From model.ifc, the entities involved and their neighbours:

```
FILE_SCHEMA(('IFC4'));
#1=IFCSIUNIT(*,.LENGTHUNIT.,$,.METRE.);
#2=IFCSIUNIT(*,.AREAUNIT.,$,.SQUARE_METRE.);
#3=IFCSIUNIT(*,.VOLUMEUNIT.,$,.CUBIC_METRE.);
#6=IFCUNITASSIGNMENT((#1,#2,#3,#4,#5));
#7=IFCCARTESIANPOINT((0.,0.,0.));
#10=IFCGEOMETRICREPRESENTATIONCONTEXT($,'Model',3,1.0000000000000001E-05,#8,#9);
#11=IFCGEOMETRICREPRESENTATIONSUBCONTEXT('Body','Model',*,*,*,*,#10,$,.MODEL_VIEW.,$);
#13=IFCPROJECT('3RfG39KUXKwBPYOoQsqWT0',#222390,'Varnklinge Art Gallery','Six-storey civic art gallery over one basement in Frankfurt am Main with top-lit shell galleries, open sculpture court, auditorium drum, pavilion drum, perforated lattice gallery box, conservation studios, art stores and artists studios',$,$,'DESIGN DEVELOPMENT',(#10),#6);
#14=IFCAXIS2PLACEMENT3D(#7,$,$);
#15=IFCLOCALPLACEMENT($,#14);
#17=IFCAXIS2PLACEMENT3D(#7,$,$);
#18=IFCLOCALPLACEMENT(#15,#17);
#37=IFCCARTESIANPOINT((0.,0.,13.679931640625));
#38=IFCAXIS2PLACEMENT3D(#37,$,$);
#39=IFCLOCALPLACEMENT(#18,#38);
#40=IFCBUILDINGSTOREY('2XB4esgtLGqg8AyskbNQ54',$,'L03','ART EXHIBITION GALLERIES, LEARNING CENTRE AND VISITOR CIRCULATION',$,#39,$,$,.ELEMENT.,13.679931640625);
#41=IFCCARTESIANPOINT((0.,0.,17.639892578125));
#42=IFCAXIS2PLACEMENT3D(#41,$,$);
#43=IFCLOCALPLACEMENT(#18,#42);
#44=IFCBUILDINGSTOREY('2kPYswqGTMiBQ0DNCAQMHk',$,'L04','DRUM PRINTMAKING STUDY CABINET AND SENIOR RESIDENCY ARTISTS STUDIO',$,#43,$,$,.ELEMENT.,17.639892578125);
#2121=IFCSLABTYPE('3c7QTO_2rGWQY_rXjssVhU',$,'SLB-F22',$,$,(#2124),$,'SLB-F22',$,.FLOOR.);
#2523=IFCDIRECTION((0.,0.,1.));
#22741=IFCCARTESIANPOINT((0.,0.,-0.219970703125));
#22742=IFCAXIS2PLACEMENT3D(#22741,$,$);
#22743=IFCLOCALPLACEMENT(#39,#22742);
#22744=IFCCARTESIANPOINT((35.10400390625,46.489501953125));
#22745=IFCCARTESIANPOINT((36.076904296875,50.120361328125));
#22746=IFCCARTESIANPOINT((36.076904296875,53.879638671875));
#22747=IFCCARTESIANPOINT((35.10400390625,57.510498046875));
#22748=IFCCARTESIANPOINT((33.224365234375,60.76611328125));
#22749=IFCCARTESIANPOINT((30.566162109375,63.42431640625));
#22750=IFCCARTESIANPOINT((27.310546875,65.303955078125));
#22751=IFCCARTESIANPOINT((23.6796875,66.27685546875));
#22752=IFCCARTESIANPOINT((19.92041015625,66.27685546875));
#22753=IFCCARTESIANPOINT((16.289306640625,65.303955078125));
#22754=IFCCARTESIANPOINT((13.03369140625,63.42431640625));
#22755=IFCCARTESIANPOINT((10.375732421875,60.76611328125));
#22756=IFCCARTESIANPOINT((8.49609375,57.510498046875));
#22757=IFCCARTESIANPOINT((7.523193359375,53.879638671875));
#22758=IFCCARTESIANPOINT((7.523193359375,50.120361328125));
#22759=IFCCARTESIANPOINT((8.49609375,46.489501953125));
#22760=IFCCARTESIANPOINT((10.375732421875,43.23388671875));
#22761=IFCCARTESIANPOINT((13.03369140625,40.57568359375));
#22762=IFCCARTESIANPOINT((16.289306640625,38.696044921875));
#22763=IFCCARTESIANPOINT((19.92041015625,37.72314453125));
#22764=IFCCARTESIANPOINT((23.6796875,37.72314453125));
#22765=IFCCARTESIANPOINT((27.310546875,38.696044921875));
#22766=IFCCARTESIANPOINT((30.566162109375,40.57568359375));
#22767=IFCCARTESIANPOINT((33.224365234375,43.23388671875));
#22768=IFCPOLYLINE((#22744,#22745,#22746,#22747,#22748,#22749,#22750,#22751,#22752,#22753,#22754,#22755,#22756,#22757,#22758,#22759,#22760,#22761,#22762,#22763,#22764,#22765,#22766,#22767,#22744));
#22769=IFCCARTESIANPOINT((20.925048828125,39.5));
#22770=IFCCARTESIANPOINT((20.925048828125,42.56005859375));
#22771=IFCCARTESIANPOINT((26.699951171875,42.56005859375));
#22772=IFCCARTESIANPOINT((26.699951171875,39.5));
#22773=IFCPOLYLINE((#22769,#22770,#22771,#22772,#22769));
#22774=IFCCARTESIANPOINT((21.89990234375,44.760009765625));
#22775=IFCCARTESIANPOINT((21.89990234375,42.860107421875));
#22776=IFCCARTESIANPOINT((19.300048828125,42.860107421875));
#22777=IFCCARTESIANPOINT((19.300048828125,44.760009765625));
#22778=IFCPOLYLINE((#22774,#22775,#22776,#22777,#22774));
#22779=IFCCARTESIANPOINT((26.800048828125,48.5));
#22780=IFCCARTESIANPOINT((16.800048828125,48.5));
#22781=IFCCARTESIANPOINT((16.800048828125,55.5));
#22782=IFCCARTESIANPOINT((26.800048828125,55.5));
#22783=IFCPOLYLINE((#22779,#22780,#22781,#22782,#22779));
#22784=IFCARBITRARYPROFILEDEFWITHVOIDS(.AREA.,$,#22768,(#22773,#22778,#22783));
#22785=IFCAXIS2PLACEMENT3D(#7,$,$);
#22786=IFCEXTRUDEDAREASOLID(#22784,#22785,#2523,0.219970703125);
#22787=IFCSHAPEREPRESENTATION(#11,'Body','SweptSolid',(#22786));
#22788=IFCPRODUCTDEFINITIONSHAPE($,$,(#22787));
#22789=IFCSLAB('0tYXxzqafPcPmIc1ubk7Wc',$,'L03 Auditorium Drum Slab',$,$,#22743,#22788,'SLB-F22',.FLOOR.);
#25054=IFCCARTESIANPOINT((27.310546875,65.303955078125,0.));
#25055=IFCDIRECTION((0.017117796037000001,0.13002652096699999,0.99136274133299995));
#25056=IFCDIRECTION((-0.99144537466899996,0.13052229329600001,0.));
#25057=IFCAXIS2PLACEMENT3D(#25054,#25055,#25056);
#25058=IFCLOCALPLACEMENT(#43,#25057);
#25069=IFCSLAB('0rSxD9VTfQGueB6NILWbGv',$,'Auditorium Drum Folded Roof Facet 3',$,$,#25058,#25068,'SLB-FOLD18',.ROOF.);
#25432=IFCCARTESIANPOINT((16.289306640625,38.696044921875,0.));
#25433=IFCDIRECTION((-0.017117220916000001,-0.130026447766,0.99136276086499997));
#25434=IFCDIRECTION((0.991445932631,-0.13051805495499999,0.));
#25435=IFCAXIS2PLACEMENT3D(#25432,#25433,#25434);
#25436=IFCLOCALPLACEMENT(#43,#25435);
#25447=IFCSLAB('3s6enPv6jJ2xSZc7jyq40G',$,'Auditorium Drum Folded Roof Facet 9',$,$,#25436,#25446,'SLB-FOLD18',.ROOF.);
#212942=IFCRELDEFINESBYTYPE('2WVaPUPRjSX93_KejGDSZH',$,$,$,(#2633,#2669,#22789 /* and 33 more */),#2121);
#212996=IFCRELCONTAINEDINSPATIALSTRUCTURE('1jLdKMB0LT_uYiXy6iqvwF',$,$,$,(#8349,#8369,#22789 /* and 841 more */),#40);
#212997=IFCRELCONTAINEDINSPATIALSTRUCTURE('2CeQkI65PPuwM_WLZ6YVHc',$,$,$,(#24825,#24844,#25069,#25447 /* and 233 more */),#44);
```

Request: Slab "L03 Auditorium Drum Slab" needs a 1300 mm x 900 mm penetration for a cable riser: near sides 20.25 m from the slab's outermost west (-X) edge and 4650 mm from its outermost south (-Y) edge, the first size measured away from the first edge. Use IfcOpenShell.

```python
import numpy as np
import ifcopenshell
import ifcopenshell.api.feature
import ifcopenshell.api.geometry
import ifcopenshell.api.root
import ifcopenshell.geom
import ifcopenshell.util.placement
import ifcopenshell.util.representation
import ifcopenshell.util.shape
import ifcopenshell.util.unit

model = ifcopenshell.open("model.ifc")
unit_scale = ifcopenshell.util.unit.calculate_unit_scale(model)
settings = ifcopenshell.geom.settings()


def volume(element):
    """Net volume in cubic metres, openings subtracted."""
    shape = ifcopenshell.geom.create_shape(settings, element)
    return ifcopenshell.util.shape.get_volume(shape.geometry)


slab = model.by_id(22789)
before = volume(slab)

# Extent in the slab's own axes, in metres. The edges named are its -X and -Y sides.
slab_shape = ifcopenshell.geom.create_shape(settings, slab)
vertices = ifcopenshell.util.shape.get_vertices(slab_shape.geometry)
x_min, y_min, bottom = vertices.min(axis=0)
top = vertices[:, 2].max()

opening = ifcopenshell.api.root.create_entity(model, ifc_class="IfcOpeningElement", name="Cable riser opening", predefined_type="OPENING")
context = ifcopenshell.util.representation.get_context(model, "Model", "Body", "MODEL_VIEW")
width, depth = 1.3, 0.9
outline = [(0.0, 0.0), (width, 0.0), (width, depth), (0.0, depth), (0.0, 0.0)]
# Overshoot both faces by 50 mm so the cut is clean.
shape = ifcopenshell.api.geometry.add_slab_representation(
    model, context=context, depth=top - bottom + 0.1, polyline=outline
)
ifcopenshell.api.geometry.assign_representation(model, product=opening, representation=shape)

matrix = ifcopenshell.util.placement.get_local_placement(slab.ObjectPlacement)
matrix[:, 3] = matrix @ np.append(np.array([x_min + 20.25, y_min + 4.65, bottom - 0.05]) / unit_scale, 1.0)
ifcopenshell.api.geometry.edit_object_placement(model, product=opening, matrix=matrix, is_si=False)
ifcopenshell.api.feature.add_feature(model, feature=opening, element=slab)

after = volume(slab)

print(f"slab volume {before:.3f} -> {after:.3f} m3")

model.write("model_edited.ifc")
```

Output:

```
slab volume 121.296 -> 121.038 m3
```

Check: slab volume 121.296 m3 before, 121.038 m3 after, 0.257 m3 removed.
